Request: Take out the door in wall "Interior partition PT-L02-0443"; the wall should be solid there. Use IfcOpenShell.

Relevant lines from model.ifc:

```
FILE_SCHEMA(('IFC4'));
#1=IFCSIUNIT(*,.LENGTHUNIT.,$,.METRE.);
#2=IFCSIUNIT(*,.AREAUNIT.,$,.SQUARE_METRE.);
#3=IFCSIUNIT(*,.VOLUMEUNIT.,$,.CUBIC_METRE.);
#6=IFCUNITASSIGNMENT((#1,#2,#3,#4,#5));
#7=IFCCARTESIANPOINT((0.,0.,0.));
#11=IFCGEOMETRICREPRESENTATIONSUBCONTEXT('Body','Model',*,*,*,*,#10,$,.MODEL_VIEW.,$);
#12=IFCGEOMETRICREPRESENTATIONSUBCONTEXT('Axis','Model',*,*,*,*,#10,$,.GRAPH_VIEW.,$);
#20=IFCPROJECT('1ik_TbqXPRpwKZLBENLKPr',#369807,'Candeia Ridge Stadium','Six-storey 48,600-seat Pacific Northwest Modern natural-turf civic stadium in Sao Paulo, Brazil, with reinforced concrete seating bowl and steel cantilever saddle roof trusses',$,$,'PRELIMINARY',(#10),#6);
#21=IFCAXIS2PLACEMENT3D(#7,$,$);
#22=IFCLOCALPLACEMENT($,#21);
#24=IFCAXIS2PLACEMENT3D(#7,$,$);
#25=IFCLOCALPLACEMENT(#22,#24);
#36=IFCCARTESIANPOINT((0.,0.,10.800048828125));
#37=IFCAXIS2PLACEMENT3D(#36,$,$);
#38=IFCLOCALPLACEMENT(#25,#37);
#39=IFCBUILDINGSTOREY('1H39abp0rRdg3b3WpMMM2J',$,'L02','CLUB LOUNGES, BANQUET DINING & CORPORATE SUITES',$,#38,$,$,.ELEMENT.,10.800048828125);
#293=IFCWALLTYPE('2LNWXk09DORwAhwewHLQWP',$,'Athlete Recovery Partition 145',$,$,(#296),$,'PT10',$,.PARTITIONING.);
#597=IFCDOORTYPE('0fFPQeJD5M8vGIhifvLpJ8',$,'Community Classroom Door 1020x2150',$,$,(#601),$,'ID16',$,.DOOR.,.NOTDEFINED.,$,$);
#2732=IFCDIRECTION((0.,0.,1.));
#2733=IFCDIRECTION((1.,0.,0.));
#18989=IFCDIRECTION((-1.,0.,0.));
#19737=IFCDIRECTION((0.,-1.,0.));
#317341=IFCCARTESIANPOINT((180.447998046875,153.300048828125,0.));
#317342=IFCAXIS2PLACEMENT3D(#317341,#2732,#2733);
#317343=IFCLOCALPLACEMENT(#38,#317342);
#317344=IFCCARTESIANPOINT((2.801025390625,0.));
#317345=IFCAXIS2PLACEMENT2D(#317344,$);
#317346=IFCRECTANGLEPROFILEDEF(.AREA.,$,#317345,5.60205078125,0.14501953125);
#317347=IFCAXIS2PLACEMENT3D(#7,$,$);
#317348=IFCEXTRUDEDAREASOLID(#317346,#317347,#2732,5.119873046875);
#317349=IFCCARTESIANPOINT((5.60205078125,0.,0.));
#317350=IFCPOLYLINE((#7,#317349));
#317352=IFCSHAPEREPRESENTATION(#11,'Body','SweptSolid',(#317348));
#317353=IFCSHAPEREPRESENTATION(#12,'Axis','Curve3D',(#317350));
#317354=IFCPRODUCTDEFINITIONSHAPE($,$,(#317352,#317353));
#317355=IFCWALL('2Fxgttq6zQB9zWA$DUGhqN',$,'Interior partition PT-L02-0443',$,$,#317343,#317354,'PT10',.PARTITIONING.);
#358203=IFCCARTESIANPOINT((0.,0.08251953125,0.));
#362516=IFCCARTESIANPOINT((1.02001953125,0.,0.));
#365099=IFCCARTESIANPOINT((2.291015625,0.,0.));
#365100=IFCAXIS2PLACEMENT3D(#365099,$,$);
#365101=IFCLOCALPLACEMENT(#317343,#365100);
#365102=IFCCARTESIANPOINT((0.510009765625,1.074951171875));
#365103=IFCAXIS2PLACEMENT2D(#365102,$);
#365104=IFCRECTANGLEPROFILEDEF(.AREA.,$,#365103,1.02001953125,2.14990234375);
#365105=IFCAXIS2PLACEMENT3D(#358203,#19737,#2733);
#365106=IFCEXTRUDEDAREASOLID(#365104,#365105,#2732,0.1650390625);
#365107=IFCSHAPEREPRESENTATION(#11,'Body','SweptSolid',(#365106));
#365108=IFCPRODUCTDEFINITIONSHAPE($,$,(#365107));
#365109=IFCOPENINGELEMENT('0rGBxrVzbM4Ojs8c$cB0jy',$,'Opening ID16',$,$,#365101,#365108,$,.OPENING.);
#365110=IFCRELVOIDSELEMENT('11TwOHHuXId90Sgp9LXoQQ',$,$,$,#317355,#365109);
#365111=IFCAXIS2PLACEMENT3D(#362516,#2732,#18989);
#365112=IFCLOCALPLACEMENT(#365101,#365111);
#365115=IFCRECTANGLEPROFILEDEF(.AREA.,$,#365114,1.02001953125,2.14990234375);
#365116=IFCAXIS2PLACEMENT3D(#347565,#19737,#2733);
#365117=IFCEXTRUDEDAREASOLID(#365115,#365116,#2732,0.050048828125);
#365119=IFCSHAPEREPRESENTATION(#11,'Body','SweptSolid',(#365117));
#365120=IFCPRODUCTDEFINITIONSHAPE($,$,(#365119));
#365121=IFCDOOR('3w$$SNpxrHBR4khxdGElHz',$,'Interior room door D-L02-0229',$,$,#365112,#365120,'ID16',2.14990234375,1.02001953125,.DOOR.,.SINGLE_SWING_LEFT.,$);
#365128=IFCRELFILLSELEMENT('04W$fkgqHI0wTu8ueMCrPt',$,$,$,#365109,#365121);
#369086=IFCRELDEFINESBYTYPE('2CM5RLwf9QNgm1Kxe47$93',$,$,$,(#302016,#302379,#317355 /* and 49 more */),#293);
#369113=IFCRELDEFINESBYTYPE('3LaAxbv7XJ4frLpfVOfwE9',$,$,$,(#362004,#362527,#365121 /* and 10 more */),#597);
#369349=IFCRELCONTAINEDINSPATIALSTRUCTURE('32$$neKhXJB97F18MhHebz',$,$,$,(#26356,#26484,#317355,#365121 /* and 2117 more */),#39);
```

```python
import ifcopenshell
import ifcopenshell.api.feature
import ifcopenshell.api.root
import ifcopenshell.geom
import ifcopenshell.util.shape

model = ifcopenshell.open("model.ifc")
settings = ifcopenshell.geom.settings()


def volume(element):
    """Net volume in cubic metres, openings subtracted."""
    shape = ifcopenshell.geom.create_shape(settings, element)
    return ifcopenshell.util.shape.get_volume(shape.geometry)


door = model.by_id(365121)
opening = door.FillsVoids[0].RelatingOpeningElement
wall = opening.VoidsElements[0].RelatingBuildingElement
before = volume(wall)

ifcopenshell.api.root.remove_product(model, product=door)
ifcopenshell.api.feature.remove_feature(model, feature=opening)

after = volume(wall)

print(f"wall volume {before:.3f} -> {after:.3f} m3")

model.write("model_edited.ifc")
```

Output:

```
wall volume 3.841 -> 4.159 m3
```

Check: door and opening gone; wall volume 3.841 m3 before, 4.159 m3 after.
